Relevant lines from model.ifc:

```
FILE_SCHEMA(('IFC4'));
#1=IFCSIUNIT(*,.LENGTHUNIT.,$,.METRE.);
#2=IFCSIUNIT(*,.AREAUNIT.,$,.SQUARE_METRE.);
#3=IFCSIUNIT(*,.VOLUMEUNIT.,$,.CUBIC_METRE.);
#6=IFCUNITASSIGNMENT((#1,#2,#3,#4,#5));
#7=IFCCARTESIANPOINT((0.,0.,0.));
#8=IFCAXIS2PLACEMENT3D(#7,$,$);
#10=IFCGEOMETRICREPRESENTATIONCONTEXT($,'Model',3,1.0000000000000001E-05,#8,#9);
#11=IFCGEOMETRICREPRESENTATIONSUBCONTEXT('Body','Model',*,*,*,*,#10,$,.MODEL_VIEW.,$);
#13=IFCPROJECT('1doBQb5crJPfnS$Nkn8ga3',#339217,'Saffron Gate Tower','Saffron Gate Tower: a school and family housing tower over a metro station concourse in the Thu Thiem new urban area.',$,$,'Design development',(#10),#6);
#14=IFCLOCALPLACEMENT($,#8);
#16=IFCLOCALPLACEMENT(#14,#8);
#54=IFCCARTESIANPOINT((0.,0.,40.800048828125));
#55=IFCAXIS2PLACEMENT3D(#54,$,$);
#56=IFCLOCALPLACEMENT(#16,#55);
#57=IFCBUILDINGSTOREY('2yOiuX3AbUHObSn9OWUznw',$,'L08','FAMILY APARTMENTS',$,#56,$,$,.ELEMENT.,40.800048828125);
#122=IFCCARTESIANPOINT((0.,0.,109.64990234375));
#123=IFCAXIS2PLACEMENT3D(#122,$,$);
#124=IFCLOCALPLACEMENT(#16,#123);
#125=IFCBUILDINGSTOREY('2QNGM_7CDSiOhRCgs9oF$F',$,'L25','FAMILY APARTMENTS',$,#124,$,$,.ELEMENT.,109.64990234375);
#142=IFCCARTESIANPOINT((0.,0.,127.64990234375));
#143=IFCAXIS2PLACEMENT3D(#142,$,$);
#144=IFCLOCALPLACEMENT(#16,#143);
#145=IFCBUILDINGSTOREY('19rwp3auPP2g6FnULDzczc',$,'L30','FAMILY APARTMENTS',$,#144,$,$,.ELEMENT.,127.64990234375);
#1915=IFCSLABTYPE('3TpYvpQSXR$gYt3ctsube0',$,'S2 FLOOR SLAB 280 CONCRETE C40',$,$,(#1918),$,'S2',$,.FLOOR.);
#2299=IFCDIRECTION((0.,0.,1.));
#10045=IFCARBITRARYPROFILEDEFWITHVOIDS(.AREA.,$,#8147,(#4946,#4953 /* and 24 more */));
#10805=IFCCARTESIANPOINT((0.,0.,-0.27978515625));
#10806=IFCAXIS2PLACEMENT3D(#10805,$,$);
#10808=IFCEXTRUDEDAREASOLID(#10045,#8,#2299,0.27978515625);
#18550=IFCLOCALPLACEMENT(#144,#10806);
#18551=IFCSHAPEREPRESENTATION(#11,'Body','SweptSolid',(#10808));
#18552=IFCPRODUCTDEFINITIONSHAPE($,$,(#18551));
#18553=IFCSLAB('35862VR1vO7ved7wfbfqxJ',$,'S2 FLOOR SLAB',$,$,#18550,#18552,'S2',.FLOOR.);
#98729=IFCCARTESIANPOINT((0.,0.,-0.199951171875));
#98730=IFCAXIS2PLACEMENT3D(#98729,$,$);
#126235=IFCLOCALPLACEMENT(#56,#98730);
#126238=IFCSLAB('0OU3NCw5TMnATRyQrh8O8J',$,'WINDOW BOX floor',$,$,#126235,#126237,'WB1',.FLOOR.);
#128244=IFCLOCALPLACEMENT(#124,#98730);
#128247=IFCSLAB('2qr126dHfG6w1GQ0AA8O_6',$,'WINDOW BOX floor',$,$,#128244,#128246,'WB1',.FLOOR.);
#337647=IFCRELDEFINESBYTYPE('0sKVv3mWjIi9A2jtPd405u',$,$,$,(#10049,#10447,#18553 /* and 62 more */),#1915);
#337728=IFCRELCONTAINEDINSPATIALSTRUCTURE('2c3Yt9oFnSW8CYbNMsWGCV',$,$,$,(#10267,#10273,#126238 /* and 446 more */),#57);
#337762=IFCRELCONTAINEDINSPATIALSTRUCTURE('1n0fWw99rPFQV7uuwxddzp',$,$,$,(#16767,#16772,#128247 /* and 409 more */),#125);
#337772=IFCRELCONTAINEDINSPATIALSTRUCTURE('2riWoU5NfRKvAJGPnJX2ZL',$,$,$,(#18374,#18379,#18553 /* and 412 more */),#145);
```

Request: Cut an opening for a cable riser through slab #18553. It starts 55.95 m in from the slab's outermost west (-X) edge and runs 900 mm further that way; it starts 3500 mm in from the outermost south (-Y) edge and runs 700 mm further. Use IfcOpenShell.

```python
import numpy as np
import ifcopenshell
import ifcopenshell.api.feature
import ifcopenshell.api.geometry
import ifcopenshell.api.root
import ifcopenshell.geom
import ifcopenshell.util.placement
import ifcopenshell.util.representation
import ifcopenshell.util.shape
import ifcopenshell.util.unit

model = ifcopenshell.open("model.ifc")
unit_scale = ifcopenshell.util.unit.calculate_unit_scale(model)
settings = ifcopenshell.geom.settings()


def volume(element):
    """Net volume in cubic metres, openings subtracted."""
    shape = ifcopenshell.geom.create_shape(settings, element)
    return ifcopenshell.util.shape.get_volume(shape.geometry)


slab = model.by_id(18553)
before = volume(slab)

# Extent in the slab's own axes, in metres. The edges named are its -X and -Y sides.
slab_shape = ifcopenshell.geom.create_shape(settings, slab)
vertices = ifcopenshell.util.shape.get_vertices(slab_shape.geometry)
x_min, y_min, bottom = vertices.min(axis=0)
top = vertices[:, 2].max()

opening = ifcopenshell.api.root.create_entity(model, ifc_class="IfcOpeningElement", name="Cable riser opening", predefined_type="OPENING")
context = ifcopenshell.util.representation.get_context(model, "Model", "Body", "MODEL_VIEW")
width, depth = 0.9, 0.7
outline = [(0.0, 0.0), (width, 0.0), (width, depth), (0.0, depth), (0.0, 0.0)]
# Overshoot both faces by 50 mm so the cut is clean.
shape = ifcopenshell.api.geometry.add_slab_representation(
    model, context=context, depth=top - bottom + 0.1, polyline=outline
)
ifcopenshell.api.geometry.assign_representation(model, product=opening, representation=shape)

matrix = ifcopenshell.util.placement.get_local_placement(slab.ObjectPlacement)
matrix[:, 3] = matrix @ np.append(np.array([x_min + 55.95, y_min + 3.5, bottom - 0.05]) / unit_scale, 1.0)
ifcopenshell.api.geometry.edit_object_placement(model, product=opening, matrix=matrix, is_si=False)
ifcopenshell.api.feature.add_feature(model, feature=opening, element=slab)

after = volume(slab)

print(f"slab volume {before:.3f} -> {after:.3f} m3")

model.write("model_updated.ifc")
```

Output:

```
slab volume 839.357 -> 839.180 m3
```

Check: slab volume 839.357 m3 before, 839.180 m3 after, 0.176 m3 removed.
